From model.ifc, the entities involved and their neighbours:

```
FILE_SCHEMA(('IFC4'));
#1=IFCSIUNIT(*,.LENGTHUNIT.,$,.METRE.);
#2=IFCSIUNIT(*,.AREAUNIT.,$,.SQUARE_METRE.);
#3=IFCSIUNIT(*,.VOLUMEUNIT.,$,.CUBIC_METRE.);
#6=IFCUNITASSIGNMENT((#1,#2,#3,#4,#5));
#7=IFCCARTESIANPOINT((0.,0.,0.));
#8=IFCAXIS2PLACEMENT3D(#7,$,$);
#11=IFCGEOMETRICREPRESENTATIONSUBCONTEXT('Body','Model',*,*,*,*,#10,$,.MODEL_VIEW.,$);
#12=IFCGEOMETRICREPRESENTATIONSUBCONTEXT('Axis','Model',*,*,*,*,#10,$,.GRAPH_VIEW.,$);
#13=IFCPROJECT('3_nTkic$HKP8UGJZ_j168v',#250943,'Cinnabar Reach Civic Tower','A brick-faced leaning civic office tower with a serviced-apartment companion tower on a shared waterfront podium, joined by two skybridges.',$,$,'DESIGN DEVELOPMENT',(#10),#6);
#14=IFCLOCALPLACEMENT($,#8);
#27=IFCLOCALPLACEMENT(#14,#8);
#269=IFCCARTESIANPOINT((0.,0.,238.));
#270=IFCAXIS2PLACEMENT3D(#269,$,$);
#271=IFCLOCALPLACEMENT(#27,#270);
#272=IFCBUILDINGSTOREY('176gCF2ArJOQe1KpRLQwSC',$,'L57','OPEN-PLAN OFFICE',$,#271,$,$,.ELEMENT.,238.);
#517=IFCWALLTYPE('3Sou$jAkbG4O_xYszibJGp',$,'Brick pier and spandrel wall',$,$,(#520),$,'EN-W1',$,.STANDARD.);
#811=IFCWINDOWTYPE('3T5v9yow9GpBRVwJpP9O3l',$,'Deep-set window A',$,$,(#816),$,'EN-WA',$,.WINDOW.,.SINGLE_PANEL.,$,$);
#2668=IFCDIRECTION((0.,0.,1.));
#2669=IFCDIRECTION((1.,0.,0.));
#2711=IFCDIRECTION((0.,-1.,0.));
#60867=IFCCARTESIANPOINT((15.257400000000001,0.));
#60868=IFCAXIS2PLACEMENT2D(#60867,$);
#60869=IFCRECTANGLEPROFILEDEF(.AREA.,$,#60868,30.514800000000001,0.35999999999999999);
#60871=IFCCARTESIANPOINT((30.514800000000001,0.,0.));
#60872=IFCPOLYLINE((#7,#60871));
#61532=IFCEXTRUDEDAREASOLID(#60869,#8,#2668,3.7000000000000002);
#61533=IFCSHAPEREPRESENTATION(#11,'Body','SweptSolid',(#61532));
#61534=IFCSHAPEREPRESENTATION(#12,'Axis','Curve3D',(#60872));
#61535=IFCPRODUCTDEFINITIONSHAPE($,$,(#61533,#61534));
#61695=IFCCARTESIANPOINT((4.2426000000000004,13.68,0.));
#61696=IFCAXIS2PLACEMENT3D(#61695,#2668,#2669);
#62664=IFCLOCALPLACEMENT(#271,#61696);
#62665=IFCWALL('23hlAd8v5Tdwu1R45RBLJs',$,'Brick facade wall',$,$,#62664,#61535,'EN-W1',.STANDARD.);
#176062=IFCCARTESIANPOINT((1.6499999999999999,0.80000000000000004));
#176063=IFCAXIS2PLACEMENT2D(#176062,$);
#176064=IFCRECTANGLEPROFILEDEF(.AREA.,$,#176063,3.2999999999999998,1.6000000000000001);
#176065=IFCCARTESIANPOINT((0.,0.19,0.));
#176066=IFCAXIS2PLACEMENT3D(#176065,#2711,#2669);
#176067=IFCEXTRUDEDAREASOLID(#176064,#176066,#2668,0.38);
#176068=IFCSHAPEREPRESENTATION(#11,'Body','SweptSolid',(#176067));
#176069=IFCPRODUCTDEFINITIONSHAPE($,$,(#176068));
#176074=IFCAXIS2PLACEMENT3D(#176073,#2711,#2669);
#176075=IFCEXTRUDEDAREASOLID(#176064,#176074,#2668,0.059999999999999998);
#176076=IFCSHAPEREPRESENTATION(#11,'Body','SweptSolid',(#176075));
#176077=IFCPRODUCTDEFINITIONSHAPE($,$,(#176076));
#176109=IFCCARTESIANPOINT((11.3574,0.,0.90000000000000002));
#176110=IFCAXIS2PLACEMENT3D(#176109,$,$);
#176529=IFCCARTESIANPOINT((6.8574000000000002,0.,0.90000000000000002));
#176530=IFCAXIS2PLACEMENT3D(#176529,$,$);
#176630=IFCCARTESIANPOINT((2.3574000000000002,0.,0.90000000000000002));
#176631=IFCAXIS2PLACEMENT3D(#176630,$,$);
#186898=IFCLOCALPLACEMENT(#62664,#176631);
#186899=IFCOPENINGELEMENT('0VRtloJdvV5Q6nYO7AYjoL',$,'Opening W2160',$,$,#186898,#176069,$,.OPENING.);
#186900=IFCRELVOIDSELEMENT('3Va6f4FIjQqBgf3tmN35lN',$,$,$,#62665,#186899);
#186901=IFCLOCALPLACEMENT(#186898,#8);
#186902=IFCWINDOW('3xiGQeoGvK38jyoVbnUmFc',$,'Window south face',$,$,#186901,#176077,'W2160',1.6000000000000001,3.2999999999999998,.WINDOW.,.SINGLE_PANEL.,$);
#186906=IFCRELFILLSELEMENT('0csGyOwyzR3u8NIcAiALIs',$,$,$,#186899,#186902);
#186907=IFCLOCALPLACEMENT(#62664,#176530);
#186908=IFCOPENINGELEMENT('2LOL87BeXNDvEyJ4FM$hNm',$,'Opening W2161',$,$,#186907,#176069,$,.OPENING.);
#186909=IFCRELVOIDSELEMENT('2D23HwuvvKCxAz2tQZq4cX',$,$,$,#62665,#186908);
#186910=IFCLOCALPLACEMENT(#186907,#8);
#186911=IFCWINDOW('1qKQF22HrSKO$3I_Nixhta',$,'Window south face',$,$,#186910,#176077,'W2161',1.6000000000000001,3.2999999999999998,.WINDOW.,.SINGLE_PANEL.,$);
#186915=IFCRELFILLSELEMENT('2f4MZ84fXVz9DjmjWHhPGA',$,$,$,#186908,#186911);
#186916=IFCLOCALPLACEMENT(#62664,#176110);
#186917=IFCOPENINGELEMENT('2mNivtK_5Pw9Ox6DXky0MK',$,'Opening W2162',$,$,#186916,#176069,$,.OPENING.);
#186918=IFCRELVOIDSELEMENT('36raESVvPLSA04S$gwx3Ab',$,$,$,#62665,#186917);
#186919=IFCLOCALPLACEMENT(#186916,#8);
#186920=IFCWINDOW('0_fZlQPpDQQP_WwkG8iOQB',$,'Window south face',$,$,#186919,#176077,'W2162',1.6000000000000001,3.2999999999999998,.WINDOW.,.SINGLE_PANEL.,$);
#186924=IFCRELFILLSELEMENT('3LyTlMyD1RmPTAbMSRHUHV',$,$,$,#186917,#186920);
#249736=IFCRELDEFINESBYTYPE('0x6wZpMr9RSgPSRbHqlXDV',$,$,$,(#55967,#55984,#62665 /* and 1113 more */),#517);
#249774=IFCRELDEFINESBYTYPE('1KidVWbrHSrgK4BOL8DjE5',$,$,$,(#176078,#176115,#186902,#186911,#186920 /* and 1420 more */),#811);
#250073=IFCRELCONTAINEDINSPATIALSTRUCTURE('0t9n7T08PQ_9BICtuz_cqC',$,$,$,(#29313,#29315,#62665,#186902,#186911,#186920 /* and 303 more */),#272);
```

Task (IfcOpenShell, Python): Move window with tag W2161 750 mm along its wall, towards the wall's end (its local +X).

```python
import ifcopenshell
import ifcopenshell.api.geometry
import ifcopenshell.util.placement
import ifcopenshell.util.unit

model = ifcopenshell.open("model.ifc")
unit_scale = ifcopenshell.util.unit.calculate_unit_scale(model)

window = model.by_id(186911)
opening = window.FillsVoids[0].RelatingOpeningElement
wall = opening.VoidsElements[0].RelatingBuildingElement

wall_matrix = ifcopenshell.util.placement.get_local_placement(wall.ObjectPlacement)
shift = wall_matrix[:3, 0] * 0.75 / unit_scale
before = ifcopenshell.util.placement.get_local_placement(window.ObjectPlacement)[:3, 3].copy()

# The window is placed relative to its opening, so it follows when the opening moves.
matrix = ifcopenshell.util.placement.get_local_placement(opening.ObjectPlacement)
matrix[:3, 3] += shift
ifcopenshell.api.geometry.edit_object_placement(
    model, product=opening, matrix=matrix, is_si=False, should_transform_children=True
)

after = ifcopenshell.util.placement.get_local_placement(window.ObjectPlacement)[:3, 3]
print("window moved by", (after - before).round(3) + 0.0)

model.write("model_updated.ifc")
```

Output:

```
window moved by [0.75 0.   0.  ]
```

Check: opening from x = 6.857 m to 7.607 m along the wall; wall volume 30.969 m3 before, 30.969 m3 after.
